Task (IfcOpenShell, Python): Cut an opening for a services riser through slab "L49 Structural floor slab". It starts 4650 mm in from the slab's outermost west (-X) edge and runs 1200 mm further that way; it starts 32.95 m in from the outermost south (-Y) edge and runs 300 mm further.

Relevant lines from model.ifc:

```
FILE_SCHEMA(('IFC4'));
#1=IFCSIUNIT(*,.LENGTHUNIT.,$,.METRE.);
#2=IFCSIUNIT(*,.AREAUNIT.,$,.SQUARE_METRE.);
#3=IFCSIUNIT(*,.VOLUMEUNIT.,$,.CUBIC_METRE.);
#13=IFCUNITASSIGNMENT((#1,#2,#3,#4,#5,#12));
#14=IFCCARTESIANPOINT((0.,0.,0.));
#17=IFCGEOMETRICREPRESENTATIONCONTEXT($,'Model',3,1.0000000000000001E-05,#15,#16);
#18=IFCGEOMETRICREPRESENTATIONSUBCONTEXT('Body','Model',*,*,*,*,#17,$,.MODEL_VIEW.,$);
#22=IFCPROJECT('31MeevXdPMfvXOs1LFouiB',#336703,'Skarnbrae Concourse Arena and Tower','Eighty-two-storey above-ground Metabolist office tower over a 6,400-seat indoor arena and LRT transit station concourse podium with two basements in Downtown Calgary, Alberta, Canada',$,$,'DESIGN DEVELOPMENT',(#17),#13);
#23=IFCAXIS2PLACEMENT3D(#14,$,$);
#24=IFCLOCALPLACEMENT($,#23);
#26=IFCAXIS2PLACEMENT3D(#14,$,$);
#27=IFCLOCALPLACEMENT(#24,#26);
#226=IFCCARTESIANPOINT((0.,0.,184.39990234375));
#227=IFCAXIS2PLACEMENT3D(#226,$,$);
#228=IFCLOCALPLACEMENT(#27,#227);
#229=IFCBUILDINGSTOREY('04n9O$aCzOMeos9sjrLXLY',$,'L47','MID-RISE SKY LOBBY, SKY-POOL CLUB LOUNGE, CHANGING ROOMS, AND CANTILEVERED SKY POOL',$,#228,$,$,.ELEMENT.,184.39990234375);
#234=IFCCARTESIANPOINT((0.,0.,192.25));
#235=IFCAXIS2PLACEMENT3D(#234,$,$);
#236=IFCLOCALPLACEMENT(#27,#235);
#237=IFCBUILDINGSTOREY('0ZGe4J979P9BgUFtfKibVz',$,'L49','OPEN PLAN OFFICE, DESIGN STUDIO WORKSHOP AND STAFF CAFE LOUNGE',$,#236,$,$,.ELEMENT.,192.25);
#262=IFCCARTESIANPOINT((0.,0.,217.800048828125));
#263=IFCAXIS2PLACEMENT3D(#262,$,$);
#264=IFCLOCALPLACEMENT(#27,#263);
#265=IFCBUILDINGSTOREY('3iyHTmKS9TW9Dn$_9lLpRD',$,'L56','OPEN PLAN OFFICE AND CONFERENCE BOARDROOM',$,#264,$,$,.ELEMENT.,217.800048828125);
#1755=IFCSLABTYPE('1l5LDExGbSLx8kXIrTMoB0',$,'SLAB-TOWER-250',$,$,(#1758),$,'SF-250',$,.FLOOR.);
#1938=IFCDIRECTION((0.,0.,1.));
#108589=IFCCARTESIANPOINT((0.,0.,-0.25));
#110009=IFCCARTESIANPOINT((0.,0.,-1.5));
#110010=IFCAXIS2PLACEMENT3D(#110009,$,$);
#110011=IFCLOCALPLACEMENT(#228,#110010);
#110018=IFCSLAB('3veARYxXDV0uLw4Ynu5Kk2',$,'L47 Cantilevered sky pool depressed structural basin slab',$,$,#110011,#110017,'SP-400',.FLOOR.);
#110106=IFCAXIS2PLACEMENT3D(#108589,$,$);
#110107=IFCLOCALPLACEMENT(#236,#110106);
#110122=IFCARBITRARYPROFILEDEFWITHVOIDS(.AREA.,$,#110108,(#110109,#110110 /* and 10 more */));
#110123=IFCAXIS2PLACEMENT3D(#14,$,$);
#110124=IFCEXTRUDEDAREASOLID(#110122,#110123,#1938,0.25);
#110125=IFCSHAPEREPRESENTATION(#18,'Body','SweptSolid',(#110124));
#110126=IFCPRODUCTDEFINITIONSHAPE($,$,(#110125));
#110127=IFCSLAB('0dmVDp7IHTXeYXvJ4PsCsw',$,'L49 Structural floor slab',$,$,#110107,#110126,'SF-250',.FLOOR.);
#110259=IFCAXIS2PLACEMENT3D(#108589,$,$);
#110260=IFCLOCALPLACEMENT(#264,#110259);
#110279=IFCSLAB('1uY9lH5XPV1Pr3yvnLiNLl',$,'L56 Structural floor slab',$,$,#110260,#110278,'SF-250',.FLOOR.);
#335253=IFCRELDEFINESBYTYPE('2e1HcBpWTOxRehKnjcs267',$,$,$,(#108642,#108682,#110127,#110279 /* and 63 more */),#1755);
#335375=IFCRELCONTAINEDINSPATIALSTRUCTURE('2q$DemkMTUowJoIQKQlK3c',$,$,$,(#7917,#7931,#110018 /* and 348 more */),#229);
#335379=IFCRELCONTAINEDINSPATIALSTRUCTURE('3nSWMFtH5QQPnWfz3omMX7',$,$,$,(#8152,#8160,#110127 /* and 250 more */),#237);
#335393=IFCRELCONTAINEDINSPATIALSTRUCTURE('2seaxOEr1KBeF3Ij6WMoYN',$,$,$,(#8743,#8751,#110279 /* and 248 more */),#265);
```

```python
import numpy as np
import ifcopenshell
import ifcopenshell.api.feature
import ifcopenshell.api.geometry
import ifcopenshell.api.root
import ifcopenshell.geom
import ifcopenshell.util.placement
import ifcopenshell.util.representation
import ifcopenshell.util.shape
import ifcopenshell.util.unit

model = ifcopenshell.open("model.ifc")
unit_scale = ifcopenshell.util.unit.calculate_unit_scale(model)
settings = ifcopenshell.geom.settings()


def volume(element):
    """Net volume in cubic metres, openings subtracted."""
    shape = ifcopenshell.geom.create_shape(settings, element)
    return ifcopenshell.util.shape.get_volume(shape.geometry)


slab = model.by_guid("0dmVDp7IHTXeYXvJ4PsCsw")
before = volume(slab)

# Extent in the slab's own axes, in metres. The edges named are its -X and -Y sides.
slab_shape = ifcopenshell.geom.create_shape(settings, slab)
vertices = ifcopenshell.util.shape.get_vertices(slab_shape.geometry)
x_min, y_min, bottom = vertices.min(axis=0)
top = vertices[:, 2].max()

opening = ifcopenshell.api.root.create_entity(model, ifc_class="IfcOpeningElement", name="Services riser opening", predefined_type="OPENING")
context = ifcopenshell.util.representation.get_context(model, "Model", "Body", "MODEL_VIEW")
width, depth = 1.2, 0.3
outline = [(0.0, 0.0), (width, 0.0), (width, depth), (0.0, depth), (0.0, 0.0)]
# Overshoot both faces by 50 mm so the cut is clean.
shape = ifcopenshell.api.geometry.add_slab_representation(
    model, context=context, depth=top - bottom + 0.1, polyline=outline
)
ifcopenshell.api.geometry.assign_representation(model, product=opening, representation=shape)

matrix = ifcopenshell.util.placement.get_local_placement(slab.ObjectPlacement)
matrix[:, 3] = matrix @ np.append(np.array([x_min + 4.65, y_min + 32.95, bottom - 0.05]) / unit_scale, 1.0)
ifcopenshell.api.geometry.edit_object_placement(model, product=opening, matrix=matrix, is_si=False)
ifcopenshell.api.feature.add_feature(model, feature=opening, element=slab)

after = volume(slab)

print(f"slab volume {before:.3f} -> {after:.3f} m3")

model.write("model_updated.ifc")
```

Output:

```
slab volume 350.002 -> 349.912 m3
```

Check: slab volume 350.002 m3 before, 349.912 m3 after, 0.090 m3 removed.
